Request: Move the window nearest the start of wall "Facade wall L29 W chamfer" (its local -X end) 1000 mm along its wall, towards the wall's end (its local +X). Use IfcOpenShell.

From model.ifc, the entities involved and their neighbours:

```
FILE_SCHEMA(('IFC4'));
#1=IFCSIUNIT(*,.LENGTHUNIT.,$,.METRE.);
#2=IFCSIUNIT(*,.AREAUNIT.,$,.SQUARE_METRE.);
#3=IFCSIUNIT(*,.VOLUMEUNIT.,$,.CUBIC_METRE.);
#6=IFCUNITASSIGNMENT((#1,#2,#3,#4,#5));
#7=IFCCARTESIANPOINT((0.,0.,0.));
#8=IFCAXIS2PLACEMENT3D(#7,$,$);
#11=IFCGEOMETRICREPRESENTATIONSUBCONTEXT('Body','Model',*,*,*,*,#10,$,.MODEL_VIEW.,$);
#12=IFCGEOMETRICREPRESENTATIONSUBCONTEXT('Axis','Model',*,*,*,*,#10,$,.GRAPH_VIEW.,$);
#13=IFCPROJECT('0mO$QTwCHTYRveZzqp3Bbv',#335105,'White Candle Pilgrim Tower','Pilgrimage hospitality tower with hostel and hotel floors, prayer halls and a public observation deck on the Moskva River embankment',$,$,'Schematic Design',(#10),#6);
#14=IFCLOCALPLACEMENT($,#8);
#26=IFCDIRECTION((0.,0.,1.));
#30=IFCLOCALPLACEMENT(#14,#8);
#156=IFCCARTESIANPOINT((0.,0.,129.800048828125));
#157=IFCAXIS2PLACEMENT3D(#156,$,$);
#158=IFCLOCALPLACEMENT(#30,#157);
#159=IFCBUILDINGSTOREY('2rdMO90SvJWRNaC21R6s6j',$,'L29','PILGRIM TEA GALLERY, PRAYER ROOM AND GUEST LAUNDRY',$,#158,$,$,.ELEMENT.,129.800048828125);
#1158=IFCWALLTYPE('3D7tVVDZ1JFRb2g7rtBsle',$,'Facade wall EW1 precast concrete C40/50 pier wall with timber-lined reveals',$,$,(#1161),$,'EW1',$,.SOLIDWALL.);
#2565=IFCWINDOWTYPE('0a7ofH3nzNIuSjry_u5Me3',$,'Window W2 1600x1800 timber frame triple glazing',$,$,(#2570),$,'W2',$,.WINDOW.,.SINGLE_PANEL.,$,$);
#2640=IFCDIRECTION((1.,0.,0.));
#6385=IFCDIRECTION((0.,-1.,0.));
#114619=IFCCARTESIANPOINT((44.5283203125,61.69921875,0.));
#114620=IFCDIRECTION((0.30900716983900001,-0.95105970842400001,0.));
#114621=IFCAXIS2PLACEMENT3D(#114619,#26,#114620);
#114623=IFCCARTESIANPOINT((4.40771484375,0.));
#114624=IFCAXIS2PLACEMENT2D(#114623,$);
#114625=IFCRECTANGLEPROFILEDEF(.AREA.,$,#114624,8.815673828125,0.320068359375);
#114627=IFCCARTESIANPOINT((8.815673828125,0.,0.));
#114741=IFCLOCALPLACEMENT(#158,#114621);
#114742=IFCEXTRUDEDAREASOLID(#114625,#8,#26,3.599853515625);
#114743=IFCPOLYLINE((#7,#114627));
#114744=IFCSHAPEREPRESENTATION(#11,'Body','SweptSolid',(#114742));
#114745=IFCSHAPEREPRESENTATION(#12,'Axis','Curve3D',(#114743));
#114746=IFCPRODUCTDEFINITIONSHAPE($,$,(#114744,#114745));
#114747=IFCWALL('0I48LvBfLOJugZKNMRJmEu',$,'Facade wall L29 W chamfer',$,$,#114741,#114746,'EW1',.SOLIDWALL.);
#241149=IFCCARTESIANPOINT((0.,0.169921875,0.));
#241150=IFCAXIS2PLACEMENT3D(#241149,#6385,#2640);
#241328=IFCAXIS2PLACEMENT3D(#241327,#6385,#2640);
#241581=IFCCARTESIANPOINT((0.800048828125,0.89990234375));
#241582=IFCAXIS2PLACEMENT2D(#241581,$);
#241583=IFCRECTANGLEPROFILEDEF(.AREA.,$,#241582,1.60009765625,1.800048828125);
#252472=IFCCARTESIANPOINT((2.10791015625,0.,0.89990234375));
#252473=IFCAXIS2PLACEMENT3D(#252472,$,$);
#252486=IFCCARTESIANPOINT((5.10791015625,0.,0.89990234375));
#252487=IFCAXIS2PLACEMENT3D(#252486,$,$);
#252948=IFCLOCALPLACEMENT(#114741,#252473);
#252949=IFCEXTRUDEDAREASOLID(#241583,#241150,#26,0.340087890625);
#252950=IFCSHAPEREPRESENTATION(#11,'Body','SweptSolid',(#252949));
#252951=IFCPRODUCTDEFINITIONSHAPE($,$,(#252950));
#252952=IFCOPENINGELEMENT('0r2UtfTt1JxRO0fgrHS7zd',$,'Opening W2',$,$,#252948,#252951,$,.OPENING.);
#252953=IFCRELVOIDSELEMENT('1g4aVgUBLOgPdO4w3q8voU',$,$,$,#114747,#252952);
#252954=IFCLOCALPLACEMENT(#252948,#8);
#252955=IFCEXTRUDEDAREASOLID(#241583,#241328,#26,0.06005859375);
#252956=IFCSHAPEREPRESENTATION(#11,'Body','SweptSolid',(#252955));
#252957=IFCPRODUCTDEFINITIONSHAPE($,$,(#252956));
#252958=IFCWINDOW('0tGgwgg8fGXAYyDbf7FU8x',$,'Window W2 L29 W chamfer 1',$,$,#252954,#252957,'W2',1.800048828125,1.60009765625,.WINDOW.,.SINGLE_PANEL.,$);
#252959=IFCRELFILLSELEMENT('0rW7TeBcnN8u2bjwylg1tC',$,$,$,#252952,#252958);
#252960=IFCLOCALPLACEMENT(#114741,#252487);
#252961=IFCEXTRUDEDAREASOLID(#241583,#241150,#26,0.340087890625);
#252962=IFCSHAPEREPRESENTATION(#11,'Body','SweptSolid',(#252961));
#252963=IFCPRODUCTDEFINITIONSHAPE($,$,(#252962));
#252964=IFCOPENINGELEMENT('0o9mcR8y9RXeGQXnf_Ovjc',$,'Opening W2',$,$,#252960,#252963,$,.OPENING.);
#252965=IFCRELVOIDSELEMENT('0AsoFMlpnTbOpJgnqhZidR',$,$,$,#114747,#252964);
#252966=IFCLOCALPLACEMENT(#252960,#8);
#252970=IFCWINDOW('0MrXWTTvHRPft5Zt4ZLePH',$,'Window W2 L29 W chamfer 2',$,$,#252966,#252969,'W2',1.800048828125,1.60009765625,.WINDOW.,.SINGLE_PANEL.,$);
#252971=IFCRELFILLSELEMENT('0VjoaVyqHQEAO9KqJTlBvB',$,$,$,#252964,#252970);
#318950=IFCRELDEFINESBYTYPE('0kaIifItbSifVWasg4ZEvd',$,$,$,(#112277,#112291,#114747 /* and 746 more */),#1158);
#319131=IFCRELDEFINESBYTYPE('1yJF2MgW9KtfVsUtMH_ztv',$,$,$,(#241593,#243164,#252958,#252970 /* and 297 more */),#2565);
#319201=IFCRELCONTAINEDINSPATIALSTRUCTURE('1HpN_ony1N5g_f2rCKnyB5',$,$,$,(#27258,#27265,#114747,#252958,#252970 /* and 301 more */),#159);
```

```python
import ifcopenshell
import ifcopenshell.api.geometry
import ifcopenshell.util.placement

model = ifcopenshell.open("model.ifc")

window = model.by_id(252958)
opening = window.FillsVoids[0].RelatingOpeningElement
wall = opening.VoidsElements[0].RelatingBuildingElement

wall_matrix = ifcopenshell.util.placement.get_local_placement(wall.ObjectPlacement)
shift = wall_matrix[:3, 0] * 1.0
before = ifcopenshell.util.placement.get_local_placement(window.ObjectPlacement)[:3, 3].copy()

# The window is placed relative to its opening, so it follows when the opening moves.
matrix = ifcopenshell.util.placement.get_local_placement(opening.ObjectPlacement)
matrix[:3, 3] += shift
ifcopenshell.api.geometry.edit_object_placement(
    model, product=opening, matrix=matrix, is_si=False, should_transform_children=True
)

after = ifcopenshell.util.placement.get_local_placement(window.ObjectPlacement)[:3, 3]
print("window moved by", (after - before).round(3) + 0.0)

model.write("model_updated.ifc")
```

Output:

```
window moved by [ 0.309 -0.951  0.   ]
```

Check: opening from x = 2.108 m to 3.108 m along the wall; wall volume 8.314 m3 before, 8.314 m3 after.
